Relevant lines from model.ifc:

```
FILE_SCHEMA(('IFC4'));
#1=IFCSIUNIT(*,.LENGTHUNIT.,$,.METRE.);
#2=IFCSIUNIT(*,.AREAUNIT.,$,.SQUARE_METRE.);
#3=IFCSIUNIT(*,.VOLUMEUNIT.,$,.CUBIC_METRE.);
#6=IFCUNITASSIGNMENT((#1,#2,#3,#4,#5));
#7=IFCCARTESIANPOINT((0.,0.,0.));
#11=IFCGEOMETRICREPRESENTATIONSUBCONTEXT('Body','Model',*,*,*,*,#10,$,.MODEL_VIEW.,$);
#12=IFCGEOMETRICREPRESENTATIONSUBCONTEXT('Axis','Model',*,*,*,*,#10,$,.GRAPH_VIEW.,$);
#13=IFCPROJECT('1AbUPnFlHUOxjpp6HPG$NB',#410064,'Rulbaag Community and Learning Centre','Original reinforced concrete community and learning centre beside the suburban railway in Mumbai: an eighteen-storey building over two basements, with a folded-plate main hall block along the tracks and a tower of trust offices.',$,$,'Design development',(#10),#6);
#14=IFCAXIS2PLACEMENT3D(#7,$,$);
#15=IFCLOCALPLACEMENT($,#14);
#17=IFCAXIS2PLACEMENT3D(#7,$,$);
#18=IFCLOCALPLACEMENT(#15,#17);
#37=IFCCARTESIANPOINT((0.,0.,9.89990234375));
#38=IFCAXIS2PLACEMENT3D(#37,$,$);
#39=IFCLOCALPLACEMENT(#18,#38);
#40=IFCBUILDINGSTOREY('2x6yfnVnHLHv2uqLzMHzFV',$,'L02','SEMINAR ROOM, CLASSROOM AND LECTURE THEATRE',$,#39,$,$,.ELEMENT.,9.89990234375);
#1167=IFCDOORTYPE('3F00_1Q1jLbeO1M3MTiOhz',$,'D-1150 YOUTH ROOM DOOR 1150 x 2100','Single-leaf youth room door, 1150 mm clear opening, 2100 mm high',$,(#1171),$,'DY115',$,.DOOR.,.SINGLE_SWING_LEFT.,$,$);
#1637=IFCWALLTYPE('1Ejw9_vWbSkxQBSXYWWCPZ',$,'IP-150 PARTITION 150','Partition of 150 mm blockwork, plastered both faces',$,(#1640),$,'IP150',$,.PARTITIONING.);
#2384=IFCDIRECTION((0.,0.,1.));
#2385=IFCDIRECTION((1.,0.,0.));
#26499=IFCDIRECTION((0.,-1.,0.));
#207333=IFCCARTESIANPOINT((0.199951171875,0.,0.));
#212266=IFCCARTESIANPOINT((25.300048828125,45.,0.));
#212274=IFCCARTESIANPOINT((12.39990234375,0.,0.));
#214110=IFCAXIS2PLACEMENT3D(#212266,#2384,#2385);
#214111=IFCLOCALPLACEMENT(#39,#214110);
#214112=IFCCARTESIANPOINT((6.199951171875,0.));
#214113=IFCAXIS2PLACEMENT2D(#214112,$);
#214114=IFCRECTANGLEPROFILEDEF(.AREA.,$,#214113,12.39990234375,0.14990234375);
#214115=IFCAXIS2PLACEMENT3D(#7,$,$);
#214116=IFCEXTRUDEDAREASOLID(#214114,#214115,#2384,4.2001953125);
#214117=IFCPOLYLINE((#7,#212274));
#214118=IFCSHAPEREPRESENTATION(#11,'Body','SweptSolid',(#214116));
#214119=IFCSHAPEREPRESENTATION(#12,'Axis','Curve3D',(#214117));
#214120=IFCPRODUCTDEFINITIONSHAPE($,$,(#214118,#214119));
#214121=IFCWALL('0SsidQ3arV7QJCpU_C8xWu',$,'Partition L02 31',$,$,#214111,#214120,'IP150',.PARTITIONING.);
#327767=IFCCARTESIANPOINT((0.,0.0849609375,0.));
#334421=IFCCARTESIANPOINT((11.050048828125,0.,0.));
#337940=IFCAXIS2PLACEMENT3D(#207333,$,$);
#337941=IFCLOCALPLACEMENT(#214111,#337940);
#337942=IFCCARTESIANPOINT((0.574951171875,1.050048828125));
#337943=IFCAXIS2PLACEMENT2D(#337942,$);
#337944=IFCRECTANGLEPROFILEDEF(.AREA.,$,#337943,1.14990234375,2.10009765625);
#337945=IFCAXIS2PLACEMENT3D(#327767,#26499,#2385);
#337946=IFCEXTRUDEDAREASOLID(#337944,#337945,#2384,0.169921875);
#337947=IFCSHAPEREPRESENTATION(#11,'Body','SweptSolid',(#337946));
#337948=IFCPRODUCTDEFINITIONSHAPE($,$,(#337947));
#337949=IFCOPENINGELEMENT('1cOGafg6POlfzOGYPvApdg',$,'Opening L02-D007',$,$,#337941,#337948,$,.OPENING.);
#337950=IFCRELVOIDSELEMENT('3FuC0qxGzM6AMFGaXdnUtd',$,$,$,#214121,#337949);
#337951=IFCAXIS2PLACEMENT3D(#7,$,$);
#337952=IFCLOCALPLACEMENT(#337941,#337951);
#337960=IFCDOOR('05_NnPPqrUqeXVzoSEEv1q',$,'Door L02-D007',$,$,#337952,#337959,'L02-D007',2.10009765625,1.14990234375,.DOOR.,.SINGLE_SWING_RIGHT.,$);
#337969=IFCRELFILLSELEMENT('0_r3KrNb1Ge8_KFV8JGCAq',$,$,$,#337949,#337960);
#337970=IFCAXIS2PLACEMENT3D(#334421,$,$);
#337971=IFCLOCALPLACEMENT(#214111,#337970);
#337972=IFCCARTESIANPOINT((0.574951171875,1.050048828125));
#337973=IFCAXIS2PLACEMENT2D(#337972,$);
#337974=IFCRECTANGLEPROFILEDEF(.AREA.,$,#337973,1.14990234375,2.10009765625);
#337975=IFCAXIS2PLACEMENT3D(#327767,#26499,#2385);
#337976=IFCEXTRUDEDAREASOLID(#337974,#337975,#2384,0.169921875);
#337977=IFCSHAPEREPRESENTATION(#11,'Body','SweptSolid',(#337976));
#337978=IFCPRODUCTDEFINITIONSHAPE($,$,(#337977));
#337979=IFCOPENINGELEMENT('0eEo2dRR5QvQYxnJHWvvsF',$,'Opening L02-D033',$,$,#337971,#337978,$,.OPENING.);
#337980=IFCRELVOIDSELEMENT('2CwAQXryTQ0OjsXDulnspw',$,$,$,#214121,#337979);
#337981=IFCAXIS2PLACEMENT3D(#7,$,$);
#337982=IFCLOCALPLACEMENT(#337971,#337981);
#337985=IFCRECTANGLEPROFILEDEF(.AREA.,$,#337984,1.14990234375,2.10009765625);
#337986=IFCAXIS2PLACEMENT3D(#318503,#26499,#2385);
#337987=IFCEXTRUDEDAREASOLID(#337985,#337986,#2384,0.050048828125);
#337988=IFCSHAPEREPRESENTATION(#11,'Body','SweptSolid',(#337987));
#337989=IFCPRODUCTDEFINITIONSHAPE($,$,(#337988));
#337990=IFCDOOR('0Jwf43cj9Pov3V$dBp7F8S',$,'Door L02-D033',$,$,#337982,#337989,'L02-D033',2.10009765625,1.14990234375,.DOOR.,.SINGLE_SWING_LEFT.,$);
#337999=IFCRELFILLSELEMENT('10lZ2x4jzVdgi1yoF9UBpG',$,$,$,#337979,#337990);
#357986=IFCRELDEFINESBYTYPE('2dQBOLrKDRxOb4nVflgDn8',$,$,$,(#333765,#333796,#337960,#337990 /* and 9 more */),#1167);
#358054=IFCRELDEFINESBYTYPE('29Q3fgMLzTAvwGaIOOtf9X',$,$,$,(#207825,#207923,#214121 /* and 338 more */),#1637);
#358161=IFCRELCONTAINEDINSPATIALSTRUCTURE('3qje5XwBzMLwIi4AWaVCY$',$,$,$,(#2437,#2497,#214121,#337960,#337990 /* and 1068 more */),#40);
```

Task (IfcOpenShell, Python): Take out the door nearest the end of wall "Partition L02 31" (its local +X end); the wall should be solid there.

```python
import ifcopenshell
import ifcopenshell.api.feature
import ifcopenshell.api.root
import ifcopenshell.geom
import ifcopenshell.util.shape

model = ifcopenshell.open("model.ifc")
settings = ifcopenshell.geom.settings()


def volume(element):
    """Net volume in cubic metres, openings subtracted."""
    shape = ifcopenshell.geom.create_shape(settings, element)
    return ifcopenshell.util.shape.get_volume(shape.geometry)


door = model.by_guid("0Jwf43cj9Pov3V$dBp7F8S")
opening = door.FillsVoids[0].RelatingOpeningElement
wall = opening.VoidsElements[0].RelatingBuildingElement
before = volume(wall)

ifcopenshell.api.root.remove_product(model, product=door)
ifcopenshell.api.feature.remove_feature(model, feature=opening)

after = volume(wall)

print(f"wall volume {before:.3f} -> {after:.3f} m3")

model.write("model_edited.ifc")
```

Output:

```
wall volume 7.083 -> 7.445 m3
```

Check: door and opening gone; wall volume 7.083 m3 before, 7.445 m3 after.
